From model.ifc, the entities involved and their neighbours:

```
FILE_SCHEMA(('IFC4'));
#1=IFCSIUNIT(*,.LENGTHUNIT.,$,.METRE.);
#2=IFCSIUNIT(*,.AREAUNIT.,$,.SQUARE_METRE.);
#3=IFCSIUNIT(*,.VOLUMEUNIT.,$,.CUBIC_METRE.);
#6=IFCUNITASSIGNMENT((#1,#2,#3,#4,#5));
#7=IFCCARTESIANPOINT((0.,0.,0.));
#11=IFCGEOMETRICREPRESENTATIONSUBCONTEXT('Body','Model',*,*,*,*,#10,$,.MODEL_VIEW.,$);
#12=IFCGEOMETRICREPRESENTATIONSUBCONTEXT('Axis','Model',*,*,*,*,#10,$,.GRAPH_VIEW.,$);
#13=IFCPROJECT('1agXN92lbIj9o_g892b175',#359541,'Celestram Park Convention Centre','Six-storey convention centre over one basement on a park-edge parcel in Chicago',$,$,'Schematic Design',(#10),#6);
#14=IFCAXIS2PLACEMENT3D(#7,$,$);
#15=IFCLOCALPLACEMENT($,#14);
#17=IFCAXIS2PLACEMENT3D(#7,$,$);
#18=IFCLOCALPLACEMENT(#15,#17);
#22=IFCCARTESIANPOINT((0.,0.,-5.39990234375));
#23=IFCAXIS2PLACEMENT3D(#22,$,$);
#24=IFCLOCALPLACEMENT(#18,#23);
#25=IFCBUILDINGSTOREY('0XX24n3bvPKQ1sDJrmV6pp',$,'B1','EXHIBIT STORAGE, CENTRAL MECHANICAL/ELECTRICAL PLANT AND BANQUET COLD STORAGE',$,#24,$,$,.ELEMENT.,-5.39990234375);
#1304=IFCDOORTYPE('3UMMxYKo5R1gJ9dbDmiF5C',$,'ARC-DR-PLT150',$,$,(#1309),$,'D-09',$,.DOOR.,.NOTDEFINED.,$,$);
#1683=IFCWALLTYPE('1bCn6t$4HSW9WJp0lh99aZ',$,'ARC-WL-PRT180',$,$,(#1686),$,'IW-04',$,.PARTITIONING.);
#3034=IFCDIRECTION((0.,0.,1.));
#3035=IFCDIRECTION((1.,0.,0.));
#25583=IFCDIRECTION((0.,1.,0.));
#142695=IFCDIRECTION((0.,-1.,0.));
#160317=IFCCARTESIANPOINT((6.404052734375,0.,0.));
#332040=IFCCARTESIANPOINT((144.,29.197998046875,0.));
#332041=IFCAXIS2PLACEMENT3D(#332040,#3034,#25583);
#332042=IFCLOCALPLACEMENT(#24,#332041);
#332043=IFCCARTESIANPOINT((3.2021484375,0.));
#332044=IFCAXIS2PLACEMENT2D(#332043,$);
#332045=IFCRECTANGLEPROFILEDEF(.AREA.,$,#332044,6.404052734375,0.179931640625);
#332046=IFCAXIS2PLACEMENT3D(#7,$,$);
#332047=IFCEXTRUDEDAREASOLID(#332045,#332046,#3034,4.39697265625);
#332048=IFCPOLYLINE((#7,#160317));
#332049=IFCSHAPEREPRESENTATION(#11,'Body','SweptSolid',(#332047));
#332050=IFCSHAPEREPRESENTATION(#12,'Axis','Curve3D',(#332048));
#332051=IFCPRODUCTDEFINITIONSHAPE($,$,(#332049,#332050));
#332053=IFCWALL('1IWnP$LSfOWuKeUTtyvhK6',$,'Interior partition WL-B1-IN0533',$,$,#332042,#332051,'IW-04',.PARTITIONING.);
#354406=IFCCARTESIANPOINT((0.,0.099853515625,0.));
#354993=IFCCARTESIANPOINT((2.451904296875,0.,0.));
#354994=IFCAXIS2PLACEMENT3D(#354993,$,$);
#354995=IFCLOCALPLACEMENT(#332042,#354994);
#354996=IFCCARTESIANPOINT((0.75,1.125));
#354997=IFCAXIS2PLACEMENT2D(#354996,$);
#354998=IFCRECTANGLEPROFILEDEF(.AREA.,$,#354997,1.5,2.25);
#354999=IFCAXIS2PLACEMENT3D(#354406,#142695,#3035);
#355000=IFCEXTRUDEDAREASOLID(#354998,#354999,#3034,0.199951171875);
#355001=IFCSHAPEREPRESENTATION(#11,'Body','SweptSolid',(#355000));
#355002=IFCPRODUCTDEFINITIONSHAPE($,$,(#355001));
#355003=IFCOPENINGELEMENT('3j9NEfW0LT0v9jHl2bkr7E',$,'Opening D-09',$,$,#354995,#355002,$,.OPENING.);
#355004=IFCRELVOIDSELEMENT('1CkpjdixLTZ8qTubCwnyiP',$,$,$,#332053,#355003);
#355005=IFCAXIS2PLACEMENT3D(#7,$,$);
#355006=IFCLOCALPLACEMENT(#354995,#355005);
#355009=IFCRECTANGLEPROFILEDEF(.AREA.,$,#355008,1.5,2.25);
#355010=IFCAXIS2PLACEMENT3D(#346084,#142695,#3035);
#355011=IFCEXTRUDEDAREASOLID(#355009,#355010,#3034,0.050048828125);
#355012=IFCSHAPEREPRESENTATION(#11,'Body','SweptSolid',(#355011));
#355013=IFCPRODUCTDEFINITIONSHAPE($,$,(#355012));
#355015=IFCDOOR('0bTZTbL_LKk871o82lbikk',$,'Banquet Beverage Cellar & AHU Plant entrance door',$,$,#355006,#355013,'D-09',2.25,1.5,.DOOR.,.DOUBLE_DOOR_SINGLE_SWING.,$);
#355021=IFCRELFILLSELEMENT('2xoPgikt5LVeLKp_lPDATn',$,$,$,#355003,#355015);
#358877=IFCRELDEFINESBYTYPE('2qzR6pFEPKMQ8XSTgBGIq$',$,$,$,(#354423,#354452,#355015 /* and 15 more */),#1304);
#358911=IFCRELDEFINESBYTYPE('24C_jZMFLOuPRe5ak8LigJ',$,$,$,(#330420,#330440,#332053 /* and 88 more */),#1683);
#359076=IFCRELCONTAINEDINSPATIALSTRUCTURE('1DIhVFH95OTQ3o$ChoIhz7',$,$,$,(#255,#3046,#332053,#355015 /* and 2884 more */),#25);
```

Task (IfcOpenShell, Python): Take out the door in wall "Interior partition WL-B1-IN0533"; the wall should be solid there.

```python
import ifcopenshell
import ifcopenshell.api.feature
import ifcopenshell.api.root
import ifcopenshell.geom
import ifcopenshell.util.shape

model = ifcopenshell.open("model.ifc")
settings = ifcopenshell.geom.settings()


def volume(element):
    """Net volume in cubic metres, openings subtracted."""
    shape = ifcopenshell.geom.create_shape(settings, element)
    return ifcopenshell.util.shape.get_volume(shape.geometry)


door = model.by_guid("0bTZTbL_LKk871o82lbikk")
opening = door.FillsVoids[0].RelatingOpeningElement
wall = opening.VoidsElements[0].RelatingBuildingElement
before = volume(wall)

ifcopenshell.api.root.remove_product(model, product=door)
ifcopenshell.api.feature.remove_feature(model, feature=opening)

after = volume(wall)

print(f"wall volume {before:.3f} -> {after:.3f} m3")

model.write("model-out.ifc")
```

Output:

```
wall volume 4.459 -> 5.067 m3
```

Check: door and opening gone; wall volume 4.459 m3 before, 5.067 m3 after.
